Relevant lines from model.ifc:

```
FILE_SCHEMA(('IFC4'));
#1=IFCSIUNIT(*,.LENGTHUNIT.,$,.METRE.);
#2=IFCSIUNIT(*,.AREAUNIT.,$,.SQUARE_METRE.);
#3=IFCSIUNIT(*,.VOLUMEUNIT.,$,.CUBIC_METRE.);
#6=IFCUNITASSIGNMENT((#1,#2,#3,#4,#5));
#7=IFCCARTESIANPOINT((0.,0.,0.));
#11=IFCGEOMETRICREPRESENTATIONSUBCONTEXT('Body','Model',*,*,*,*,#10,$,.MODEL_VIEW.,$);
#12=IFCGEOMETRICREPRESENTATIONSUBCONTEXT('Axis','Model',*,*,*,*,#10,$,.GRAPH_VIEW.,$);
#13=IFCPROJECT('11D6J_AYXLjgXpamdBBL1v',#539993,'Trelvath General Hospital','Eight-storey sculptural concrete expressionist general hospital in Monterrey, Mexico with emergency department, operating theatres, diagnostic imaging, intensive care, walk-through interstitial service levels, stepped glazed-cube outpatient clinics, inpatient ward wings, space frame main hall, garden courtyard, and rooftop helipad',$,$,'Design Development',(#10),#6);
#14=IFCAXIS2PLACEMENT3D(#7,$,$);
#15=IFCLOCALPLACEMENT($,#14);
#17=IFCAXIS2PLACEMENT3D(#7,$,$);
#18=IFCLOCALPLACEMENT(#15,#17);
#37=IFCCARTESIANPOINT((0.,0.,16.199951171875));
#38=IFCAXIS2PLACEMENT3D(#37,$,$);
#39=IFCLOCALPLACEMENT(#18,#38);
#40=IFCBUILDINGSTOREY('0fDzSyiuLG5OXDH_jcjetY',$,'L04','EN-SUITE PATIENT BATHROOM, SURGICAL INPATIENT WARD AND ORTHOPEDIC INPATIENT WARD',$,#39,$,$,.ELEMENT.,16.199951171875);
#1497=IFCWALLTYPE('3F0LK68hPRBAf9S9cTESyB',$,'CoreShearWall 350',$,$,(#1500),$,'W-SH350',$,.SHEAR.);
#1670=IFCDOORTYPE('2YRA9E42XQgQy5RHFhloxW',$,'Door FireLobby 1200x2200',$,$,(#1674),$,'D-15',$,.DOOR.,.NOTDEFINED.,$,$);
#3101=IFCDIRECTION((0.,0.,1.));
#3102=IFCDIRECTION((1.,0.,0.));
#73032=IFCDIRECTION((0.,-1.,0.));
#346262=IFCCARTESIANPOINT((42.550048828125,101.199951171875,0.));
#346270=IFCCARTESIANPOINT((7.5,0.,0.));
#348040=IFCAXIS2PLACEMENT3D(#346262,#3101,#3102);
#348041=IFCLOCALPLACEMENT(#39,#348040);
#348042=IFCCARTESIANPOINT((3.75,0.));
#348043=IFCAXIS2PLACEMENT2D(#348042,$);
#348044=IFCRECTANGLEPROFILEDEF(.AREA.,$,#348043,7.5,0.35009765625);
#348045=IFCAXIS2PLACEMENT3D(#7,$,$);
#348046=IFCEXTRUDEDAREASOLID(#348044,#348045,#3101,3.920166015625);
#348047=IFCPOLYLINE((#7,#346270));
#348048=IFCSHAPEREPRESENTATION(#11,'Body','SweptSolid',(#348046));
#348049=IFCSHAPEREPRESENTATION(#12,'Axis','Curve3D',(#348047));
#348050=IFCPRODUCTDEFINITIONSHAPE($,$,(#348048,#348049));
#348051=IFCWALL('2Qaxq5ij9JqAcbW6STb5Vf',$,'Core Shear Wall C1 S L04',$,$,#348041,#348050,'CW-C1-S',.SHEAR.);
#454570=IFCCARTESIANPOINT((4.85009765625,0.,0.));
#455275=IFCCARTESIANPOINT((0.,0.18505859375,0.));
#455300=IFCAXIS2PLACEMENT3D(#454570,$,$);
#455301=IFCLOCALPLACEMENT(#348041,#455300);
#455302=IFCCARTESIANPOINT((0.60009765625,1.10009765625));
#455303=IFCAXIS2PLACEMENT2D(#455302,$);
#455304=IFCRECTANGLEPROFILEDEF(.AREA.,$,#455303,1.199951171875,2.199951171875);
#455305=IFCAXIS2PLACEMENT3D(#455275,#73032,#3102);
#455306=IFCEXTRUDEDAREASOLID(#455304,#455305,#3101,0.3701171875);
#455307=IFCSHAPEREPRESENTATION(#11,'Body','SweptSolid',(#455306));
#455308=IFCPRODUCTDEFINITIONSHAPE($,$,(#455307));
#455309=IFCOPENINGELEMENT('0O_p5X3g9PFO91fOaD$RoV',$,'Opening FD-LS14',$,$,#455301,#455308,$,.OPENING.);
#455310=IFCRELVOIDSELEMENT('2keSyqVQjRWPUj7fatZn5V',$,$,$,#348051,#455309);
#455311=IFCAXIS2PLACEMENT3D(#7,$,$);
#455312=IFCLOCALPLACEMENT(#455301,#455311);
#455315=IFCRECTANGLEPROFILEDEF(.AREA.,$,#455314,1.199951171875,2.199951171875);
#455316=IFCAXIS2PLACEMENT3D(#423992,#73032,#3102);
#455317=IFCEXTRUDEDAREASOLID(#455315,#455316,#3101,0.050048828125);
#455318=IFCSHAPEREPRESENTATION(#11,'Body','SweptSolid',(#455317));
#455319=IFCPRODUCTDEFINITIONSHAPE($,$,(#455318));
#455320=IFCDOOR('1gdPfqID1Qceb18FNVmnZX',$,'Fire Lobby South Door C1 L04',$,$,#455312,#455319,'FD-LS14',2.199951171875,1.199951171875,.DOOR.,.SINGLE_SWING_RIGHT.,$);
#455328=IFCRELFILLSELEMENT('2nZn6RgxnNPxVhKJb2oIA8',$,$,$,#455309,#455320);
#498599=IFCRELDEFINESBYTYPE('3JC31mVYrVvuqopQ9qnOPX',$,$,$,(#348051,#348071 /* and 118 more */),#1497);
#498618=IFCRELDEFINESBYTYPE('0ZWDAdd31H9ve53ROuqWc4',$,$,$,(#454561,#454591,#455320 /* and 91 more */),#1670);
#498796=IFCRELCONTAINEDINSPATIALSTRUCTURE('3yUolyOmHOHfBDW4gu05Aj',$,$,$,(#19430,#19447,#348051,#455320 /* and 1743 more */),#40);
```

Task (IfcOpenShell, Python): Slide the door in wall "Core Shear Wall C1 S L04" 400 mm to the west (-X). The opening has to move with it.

```python
import ifcopenshell
import ifcopenshell.api.geometry
import ifcopenshell.util.placement
import ifcopenshell.util.unit

model = ifcopenshell.open("model.ifc")
unit_scale = ifcopenshell.util.unit.calculate_unit_scale(model)

door = model.by_id(455320)
opening = door.FillsVoids[0].RelatingOpeningElement
wall = opening.VoidsElements[0].RelatingBuildingElement

wall_matrix = ifcopenshell.util.placement.get_local_placement(wall.ObjectPlacement)
shift = wall_matrix[:3, 0] * -0.4 / unit_scale
before = ifcopenshell.util.placement.get_local_placement(door.ObjectPlacement)[:3, 3].copy()

# The door is placed relative to its opening, so it follows when the opening moves.
matrix = ifcopenshell.util.placement.get_local_placement(opening.ObjectPlacement)
matrix[:3, 3] += shift
ifcopenshell.api.geometry.edit_object_placement(
    model, product=opening, matrix=matrix, is_si=False, should_transform_children=True
)

after = ifcopenshell.util.placement.get_local_placement(door.ObjectPlacement)[:3, 3]
print("door moved by", (after - before).round(3) + 0.0)

model.write("model_edited.ifc")
```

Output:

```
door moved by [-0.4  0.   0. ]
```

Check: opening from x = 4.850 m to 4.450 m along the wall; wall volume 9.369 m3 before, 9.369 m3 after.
